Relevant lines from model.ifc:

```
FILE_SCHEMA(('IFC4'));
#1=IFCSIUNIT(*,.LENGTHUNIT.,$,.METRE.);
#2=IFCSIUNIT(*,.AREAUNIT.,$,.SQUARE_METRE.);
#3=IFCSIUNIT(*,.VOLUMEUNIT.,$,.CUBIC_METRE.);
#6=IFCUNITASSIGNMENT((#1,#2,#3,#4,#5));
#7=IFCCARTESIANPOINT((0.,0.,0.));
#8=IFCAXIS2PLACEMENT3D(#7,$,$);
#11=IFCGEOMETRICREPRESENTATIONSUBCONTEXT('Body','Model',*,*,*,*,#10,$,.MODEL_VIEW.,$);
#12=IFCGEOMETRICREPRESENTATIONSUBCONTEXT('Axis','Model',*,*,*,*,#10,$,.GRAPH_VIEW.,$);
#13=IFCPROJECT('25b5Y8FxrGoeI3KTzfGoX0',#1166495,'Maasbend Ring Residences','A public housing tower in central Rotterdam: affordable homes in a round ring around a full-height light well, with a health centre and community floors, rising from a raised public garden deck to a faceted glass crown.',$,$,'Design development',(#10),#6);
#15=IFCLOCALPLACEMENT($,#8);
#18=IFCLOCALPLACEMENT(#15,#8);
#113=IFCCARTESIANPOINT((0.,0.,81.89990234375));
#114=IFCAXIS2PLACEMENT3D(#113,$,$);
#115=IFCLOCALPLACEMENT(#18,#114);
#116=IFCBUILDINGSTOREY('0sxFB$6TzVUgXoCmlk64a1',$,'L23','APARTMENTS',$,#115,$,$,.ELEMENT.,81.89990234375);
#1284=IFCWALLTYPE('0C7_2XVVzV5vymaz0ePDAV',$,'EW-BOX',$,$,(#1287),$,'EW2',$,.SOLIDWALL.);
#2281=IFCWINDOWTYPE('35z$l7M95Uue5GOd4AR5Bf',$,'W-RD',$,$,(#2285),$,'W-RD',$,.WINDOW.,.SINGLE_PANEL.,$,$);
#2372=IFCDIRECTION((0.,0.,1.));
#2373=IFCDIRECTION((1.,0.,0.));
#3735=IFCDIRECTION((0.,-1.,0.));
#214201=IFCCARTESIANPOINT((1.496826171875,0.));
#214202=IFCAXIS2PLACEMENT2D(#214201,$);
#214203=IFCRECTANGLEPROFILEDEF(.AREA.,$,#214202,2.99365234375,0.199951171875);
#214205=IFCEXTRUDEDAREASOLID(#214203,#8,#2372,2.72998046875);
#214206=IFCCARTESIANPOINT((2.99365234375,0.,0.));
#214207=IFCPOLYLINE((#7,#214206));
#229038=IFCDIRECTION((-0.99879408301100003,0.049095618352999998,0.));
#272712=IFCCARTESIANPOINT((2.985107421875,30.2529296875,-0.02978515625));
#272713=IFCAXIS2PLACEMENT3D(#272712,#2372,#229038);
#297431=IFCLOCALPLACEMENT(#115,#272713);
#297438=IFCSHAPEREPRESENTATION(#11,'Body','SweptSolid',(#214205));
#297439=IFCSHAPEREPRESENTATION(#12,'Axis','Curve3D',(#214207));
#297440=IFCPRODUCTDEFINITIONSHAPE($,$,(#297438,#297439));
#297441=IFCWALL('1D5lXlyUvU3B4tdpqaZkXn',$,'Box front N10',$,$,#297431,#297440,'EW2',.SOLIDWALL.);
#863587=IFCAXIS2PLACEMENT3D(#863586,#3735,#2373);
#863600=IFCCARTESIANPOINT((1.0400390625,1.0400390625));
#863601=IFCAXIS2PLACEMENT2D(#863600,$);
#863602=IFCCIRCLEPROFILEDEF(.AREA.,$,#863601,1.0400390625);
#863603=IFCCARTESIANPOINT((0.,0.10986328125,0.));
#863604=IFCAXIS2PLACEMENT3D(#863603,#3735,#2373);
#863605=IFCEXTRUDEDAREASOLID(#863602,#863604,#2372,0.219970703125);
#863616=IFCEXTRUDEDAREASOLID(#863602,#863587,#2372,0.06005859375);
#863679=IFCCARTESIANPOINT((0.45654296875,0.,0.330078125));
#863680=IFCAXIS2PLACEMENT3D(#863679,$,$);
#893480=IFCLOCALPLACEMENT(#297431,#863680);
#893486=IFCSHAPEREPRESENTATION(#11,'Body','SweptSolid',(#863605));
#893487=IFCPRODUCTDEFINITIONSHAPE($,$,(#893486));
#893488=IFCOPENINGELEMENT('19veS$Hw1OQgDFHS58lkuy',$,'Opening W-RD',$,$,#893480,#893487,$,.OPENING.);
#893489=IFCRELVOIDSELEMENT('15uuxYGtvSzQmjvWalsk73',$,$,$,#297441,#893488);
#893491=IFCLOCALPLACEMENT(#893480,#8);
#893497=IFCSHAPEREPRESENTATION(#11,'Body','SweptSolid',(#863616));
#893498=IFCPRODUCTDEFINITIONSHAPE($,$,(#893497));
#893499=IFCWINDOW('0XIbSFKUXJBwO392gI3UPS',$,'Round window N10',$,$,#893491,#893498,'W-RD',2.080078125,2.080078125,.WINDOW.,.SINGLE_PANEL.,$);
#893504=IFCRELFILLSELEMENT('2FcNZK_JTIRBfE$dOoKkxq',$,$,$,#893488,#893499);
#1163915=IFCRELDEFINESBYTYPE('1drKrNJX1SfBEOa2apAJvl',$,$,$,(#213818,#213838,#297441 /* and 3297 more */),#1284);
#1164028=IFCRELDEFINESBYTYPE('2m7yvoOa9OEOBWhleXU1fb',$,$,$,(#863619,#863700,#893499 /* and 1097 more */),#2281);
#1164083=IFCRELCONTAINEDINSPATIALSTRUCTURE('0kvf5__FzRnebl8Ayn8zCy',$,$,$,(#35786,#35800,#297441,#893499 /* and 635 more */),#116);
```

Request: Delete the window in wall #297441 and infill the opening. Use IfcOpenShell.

```python
import ifcopenshell
import ifcopenshell.api.feature
import ifcopenshell.api.root
import ifcopenshell.geom
import ifcopenshell.util.shape

model = ifcopenshell.open("model.ifc")
settings = ifcopenshell.geom.settings()


def volume(element):
    """Net volume in cubic metres, openings subtracted."""
    shape = ifcopenshell.geom.create_shape(settings, element)
    return ifcopenshell.util.shape.get_volume(shape.geometry)


window = model.by_id(893499)
opening = window.FillsVoids[0].RelatingOpeningElement
wall = opening.VoidsElements[0].RelatingBuildingElement
before = volume(wall)

ifcopenshell.api.root.remove_product(model, product=window)
ifcopenshell.api.feature.remove_feature(model, feature=opening)

after = volume(wall)

print(f"wall volume {before:.3f} -> {after:.3f} m3")

model.write("model_rev.ifc")
```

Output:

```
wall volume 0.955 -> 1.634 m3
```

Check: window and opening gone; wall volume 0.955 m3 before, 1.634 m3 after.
